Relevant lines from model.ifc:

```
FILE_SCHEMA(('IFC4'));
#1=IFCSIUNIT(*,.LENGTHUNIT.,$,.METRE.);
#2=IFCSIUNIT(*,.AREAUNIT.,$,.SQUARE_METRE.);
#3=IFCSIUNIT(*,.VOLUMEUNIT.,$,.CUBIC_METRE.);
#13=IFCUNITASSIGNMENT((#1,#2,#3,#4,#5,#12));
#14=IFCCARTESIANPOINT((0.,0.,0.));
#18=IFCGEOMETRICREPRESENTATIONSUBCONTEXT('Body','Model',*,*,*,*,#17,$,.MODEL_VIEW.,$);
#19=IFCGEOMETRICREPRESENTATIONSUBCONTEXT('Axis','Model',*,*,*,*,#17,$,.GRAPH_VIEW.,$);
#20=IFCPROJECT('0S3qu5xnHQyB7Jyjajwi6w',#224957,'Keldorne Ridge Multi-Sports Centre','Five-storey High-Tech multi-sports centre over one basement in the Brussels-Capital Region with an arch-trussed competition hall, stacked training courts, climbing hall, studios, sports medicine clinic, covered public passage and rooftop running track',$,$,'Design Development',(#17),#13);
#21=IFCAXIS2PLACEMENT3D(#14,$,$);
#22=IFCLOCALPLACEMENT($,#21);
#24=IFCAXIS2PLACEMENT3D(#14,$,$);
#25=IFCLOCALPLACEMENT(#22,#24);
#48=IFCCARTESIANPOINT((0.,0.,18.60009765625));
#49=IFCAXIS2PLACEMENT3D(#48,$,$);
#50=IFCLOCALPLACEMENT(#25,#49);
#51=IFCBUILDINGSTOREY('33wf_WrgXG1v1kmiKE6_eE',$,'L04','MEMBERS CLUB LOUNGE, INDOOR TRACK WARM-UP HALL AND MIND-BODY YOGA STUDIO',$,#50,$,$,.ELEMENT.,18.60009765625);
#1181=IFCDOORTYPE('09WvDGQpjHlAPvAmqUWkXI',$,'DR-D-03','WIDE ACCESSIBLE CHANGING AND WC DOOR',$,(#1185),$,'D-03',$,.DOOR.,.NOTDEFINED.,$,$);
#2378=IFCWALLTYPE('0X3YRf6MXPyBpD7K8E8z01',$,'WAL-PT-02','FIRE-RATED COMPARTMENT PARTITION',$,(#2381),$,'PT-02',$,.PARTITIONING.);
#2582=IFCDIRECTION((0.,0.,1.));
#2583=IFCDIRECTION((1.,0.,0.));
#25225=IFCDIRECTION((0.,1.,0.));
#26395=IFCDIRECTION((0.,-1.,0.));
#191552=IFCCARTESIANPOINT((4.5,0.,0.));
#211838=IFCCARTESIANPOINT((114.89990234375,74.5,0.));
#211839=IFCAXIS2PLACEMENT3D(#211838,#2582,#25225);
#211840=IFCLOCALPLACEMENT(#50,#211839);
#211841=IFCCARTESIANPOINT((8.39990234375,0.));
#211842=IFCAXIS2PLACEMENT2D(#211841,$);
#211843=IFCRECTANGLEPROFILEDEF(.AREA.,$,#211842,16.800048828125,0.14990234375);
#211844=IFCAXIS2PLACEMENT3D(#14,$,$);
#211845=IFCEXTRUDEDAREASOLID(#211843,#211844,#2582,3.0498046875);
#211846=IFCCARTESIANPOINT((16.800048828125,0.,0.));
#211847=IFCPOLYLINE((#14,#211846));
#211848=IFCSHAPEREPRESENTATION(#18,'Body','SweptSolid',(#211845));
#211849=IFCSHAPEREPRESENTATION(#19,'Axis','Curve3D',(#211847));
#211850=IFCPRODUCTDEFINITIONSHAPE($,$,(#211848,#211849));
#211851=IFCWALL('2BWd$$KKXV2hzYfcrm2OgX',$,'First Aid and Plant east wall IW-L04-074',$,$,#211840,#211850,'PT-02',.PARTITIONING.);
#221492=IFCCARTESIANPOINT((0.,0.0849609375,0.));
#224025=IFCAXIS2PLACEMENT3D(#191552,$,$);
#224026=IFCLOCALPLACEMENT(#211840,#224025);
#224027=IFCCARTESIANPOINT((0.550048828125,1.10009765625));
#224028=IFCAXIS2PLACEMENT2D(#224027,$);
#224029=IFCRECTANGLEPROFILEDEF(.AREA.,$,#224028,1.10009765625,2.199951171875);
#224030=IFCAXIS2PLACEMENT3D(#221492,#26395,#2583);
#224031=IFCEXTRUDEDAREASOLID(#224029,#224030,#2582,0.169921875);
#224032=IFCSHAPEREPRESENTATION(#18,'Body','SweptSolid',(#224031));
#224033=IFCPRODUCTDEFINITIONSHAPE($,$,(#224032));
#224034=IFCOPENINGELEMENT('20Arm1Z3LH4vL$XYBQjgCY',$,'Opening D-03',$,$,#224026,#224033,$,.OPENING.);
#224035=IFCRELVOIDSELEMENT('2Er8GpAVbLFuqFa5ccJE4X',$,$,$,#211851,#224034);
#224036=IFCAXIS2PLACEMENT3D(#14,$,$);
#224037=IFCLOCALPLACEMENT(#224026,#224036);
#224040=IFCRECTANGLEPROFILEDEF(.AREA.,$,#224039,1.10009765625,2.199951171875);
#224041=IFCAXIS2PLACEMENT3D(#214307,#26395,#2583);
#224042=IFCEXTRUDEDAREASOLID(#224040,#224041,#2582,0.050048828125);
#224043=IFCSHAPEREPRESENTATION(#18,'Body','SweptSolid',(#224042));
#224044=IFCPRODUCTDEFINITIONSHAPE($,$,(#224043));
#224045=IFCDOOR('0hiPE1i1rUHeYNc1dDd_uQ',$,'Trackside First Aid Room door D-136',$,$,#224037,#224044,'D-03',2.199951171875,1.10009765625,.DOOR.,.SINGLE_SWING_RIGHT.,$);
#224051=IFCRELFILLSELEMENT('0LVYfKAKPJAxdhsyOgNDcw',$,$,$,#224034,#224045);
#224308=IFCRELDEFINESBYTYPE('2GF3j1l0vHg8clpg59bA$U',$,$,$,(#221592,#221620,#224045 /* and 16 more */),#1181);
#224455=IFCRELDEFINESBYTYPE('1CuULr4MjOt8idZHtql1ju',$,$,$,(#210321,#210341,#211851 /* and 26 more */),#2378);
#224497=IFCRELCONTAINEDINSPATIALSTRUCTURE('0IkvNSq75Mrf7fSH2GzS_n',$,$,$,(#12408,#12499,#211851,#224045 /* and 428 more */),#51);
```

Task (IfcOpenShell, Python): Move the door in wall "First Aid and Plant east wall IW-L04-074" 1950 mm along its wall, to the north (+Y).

```python
import ifcopenshell
import ifcopenshell.api.geometry
import ifcopenshell.util.placement

model = ifcopenshell.open("model.ifc")

door = model.by_id(224045)
opening = door.FillsVoids[0].RelatingOpeningElement
wall = opening.VoidsElements[0].RelatingBuildingElement

wall_matrix = ifcopenshell.util.placement.get_local_placement(wall.ObjectPlacement)
shift = wall_matrix[:3, 0] * 1.95
before = ifcopenshell.util.placement.get_local_placement(door.ObjectPlacement)[:3, 3].copy()

# The door is placed relative to its opening, so it follows when the opening moves.
matrix = ifcopenshell.util.placement.get_local_placement(opening.ObjectPlacement)
matrix[:3, 3] += shift
ifcopenshell.api.geometry.edit_object_placement(
    model, product=opening, matrix=matrix, is_si=False, should_transform_children=True
)

after = ifcopenshell.util.placement.get_local_placement(door.ObjectPlacement)[:3, 3]
print("door moved by", (after - before).round(3) + 0.0)

model.write("model_updated.ifc")
```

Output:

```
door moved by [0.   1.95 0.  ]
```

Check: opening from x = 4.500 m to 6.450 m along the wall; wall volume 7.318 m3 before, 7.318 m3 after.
